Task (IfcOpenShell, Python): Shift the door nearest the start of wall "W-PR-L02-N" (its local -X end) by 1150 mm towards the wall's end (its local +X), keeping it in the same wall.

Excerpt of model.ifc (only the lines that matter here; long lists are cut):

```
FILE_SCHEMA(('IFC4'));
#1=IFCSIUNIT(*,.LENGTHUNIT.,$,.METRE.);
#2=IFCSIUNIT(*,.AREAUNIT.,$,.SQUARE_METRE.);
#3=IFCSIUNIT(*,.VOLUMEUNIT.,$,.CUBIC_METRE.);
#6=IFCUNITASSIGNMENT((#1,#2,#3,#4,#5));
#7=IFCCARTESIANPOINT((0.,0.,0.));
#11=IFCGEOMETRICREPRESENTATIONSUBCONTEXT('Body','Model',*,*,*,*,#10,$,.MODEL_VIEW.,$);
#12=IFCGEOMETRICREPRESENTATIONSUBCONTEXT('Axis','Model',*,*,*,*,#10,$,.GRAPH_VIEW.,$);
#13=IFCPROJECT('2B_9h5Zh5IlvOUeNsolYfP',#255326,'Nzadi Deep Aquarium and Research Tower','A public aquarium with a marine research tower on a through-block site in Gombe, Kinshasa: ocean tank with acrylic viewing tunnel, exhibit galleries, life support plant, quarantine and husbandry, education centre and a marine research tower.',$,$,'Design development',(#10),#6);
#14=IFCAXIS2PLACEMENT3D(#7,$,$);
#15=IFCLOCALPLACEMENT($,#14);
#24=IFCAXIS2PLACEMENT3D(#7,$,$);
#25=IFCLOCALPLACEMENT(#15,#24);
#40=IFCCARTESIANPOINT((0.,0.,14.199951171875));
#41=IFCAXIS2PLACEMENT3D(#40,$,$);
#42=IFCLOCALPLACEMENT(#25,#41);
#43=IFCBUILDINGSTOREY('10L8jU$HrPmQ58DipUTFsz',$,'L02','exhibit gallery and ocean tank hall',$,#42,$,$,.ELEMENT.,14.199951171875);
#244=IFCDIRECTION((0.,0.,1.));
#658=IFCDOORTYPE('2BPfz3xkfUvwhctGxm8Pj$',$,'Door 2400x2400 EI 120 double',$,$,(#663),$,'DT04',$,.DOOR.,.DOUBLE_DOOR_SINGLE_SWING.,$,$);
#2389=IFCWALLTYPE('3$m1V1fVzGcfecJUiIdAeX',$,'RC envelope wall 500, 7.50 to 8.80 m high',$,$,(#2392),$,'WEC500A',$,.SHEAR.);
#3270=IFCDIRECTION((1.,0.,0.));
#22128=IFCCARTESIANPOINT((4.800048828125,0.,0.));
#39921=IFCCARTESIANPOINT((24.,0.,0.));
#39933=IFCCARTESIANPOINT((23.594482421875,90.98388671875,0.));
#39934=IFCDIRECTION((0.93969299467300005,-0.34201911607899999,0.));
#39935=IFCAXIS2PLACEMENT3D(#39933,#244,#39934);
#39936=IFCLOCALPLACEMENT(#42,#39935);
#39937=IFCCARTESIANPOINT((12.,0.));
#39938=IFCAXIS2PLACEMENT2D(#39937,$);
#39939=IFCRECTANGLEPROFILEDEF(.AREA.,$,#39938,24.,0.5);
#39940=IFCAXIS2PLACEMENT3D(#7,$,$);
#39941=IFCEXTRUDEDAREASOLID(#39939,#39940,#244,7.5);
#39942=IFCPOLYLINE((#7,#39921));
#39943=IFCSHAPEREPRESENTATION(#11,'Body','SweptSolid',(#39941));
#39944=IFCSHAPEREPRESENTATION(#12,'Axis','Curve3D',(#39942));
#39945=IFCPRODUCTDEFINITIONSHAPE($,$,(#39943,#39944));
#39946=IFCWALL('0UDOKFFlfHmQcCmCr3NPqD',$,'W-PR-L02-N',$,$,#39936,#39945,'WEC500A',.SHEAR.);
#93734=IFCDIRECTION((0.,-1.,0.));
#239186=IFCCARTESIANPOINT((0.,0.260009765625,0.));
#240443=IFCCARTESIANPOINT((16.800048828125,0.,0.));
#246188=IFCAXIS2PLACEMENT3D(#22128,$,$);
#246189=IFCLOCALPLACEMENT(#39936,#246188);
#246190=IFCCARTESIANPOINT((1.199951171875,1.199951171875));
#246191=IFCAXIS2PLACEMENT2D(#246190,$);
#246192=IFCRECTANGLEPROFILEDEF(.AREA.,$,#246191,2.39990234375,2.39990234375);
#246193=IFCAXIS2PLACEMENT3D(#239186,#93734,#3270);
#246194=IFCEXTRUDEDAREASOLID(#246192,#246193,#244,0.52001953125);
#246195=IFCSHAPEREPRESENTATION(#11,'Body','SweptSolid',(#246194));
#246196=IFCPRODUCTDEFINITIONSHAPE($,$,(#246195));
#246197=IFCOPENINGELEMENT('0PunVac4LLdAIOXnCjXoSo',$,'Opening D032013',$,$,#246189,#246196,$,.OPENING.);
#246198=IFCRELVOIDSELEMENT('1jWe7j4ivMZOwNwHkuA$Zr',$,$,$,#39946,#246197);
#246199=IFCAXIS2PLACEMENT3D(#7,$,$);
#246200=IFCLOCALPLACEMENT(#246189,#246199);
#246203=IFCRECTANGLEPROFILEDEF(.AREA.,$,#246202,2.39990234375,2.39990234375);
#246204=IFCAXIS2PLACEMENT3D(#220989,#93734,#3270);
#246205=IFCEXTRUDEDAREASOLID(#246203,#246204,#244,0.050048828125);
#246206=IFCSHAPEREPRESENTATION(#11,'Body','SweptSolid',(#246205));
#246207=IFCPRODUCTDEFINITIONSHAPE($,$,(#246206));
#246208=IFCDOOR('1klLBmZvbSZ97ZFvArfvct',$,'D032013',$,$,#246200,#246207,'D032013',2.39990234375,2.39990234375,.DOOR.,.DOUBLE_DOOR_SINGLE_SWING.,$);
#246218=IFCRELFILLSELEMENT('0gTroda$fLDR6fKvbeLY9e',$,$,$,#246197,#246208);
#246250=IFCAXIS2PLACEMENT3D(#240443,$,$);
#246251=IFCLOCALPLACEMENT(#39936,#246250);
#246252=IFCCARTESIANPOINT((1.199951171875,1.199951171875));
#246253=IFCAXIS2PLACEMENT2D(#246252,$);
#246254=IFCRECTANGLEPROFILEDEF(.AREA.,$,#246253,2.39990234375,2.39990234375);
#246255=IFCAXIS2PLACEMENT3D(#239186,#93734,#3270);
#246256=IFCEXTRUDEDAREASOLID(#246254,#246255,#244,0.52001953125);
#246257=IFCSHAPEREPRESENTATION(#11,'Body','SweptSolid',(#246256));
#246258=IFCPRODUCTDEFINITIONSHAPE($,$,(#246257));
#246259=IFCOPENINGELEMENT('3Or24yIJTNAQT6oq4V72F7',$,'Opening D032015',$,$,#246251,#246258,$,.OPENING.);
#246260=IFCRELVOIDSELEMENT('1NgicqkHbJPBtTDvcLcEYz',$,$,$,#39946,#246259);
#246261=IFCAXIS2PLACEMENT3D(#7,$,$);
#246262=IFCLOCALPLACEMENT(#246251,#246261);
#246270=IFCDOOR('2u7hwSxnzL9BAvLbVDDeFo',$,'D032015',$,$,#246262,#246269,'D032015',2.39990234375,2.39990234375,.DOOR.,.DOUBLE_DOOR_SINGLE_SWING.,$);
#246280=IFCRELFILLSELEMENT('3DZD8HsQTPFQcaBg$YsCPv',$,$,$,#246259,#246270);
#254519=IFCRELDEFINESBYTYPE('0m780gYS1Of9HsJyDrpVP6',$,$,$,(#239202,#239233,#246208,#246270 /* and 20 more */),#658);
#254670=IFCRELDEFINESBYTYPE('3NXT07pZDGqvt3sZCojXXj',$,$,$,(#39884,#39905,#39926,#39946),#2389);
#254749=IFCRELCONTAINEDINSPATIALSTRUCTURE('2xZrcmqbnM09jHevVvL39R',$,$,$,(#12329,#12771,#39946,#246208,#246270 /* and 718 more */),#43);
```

```python
import ifcopenshell
import ifcopenshell.api.geometry
import ifcopenshell.util.placement
import ifcopenshell.util.unit

model = ifcopenshell.open("model.ifc")
unit_scale = ifcopenshell.util.unit.calculate_unit_scale(model)

door = model.by_guid("1klLBmZvbSZ97ZFvArfvct")
opening = door.FillsVoids[0].RelatingOpeningElement
wall = opening.VoidsElements[0].RelatingBuildingElement

wall_matrix = ifcopenshell.util.placement.get_local_placement(wall.ObjectPlacement)
shift = wall_matrix[:3, 0] * 1.15 / unit_scale
before = ifcopenshell.util.placement.get_local_placement(door.ObjectPlacement)[:3, 3].copy()

# The door is placed relative to its opening, so it follows when the opening moves.
matrix = ifcopenshell.util.placement.get_local_placement(opening.ObjectPlacement)
matrix[:3, 3] += shift
ifcopenshell.api.geometry.edit_object_placement(
    model, product=opening, matrix=matrix, is_si=False, should_transform_children=True
)

after = ifcopenshell.util.placement.get_local_placement(door.ObjectPlacement)[:3, 3]
print("door moved by", (after - before).round(3) + 0.0)

model.write("model_v2.ifc")
```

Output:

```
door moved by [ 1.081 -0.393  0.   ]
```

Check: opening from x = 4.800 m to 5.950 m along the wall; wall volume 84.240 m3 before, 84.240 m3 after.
